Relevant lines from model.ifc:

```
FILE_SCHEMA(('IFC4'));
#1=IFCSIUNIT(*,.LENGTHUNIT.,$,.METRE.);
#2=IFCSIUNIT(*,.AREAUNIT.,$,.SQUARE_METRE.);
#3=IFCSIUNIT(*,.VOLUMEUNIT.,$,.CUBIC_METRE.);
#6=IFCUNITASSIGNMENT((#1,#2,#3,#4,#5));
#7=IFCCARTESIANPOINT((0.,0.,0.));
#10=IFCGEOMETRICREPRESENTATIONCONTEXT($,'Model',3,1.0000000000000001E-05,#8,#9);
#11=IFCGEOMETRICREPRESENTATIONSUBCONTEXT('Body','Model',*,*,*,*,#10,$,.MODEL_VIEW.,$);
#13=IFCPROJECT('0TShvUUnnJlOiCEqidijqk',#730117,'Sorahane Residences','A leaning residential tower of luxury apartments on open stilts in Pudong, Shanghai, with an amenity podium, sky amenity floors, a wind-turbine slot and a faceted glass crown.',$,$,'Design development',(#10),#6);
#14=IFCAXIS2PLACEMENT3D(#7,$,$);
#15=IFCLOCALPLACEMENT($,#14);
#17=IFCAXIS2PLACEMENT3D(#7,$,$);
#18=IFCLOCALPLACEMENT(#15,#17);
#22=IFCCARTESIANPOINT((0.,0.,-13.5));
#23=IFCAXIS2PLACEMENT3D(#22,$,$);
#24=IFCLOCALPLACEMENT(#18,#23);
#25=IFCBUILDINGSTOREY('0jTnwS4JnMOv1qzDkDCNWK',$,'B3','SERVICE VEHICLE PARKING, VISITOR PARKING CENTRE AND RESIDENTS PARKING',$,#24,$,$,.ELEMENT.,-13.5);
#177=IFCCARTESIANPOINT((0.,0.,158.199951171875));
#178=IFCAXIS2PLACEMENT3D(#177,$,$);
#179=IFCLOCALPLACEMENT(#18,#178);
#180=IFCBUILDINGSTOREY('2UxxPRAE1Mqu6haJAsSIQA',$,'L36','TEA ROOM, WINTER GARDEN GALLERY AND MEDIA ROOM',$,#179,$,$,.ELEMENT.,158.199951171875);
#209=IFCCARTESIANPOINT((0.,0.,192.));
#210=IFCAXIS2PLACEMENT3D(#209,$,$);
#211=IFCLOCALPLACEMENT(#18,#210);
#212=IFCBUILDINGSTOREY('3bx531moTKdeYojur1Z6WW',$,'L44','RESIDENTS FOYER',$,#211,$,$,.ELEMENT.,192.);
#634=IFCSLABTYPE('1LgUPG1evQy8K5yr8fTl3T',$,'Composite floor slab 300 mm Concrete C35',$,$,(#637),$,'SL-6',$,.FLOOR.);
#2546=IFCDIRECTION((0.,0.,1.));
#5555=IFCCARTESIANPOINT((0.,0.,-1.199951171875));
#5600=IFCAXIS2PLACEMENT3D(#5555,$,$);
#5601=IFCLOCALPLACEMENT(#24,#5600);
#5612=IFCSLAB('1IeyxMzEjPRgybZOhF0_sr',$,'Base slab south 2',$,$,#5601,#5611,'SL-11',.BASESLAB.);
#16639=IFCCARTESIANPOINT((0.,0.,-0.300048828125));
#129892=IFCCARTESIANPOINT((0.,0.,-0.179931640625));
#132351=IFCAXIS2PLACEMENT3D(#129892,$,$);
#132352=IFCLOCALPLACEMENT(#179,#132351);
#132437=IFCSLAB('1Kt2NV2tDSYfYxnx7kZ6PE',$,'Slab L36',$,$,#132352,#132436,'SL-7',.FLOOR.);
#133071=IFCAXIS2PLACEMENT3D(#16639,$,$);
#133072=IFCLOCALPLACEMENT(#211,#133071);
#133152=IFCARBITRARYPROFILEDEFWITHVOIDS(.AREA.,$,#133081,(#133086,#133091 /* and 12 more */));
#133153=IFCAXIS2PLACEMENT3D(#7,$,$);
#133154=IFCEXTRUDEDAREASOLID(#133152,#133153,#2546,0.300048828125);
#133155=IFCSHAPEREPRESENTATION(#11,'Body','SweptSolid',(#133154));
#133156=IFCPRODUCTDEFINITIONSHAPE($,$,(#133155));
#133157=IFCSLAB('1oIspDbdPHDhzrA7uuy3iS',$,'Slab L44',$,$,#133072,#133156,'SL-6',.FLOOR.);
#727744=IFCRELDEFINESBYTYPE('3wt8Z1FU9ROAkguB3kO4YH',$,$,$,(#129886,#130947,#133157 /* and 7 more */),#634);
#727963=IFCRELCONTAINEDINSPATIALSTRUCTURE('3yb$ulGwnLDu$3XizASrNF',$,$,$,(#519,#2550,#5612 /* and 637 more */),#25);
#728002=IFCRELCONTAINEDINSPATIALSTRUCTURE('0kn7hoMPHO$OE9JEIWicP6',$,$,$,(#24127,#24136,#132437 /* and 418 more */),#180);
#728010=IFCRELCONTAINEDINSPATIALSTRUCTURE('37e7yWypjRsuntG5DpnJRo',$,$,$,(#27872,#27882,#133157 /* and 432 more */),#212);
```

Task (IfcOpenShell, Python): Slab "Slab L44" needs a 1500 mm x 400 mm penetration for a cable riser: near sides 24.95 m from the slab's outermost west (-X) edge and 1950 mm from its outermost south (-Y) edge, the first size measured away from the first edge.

```python
import numpy as np
import ifcopenshell
import ifcopenshell.api.feature
import ifcopenshell.api.geometry
import ifcopenshell.api.root
import ifcopenshell.geom
import ifcopenshell.util.placement
import ifcopenshell.util.representation
import ifcopenshell.util.shape
import ifcopenshell.util.unit

model = ifcopenshell.open("model.ifc")
unit_scale = ifcopenshell.util.unit.calculate_unit_scale(model)
settings = ifcopenshell.geom.settings()


def volume(element):
    """Net volume in cubic metres, openings subtracted."""
    shape = ifcopenshell.geom.create_shape(settings, element)
    return ifcopenshell.util.shape.get_volume(shape.geometry)


slab = model.by_guid("1oIspDbdPHDhzrA7uuy3iS")
before = volume(slab)

# Extent in the slab's own axes, in metres. The edges named are its -X and -Y sides.
slab_shape = ifcopenshell.geom.create_shape(settings, slab)
vertices = ifcopenshell.util.shape.get_vertices(slab_shape.geometry)
x_min, y_min, bottom = vertices.min(axis=0)
top = vertices[:, 2].max()

opening = ifcopenshell.api.root.create_entity(model, ifc_class="IfcOpeningElement", name="Cable riser opening", predefined_type="OPENING")
context = ifcopenshell.util.representation.get_context(model, "Model", "Body", "MODEL_VIEW")
width, depth = 1.5, 0.4
outline = [(0.0, 0.0), (width, 0.0), (width, depth), (0.0, depth), (0.0, 0.0)]
# Overshoot both faces by 50 mm so the cut is clean.
shape = ifcopenshell.api.geometry.add_slab_representation(
    model, context=context, depth=top - bottom + 0.1, polyline=outline
)
ifcopenshell.api.geometry.assign_representation(model, product=opening, representation=shape)

matrix = ifcopenshell.util.placement.get_local_placement(slab.ObjectPlacement)
matrix[:, 3] = matrix @ np.append(np.array([x_min + 24.95, y_min + 1.95, bottom - 0.05]) / unit_scale, 1.0)
ifcopenshell.api.geometry.edit_object_placement(model, product=opening, matrix=matrix, is_si=False)
ifcopenshell.api.feature.add_feature(model, feature=opening, element=slab)

after = volume(slab)

print(f"slab volume {before:.3f} -> {after:.3f} m3")

model.write("model_rev.ifc")
```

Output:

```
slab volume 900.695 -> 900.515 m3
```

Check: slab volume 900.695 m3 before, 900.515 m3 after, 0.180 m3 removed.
